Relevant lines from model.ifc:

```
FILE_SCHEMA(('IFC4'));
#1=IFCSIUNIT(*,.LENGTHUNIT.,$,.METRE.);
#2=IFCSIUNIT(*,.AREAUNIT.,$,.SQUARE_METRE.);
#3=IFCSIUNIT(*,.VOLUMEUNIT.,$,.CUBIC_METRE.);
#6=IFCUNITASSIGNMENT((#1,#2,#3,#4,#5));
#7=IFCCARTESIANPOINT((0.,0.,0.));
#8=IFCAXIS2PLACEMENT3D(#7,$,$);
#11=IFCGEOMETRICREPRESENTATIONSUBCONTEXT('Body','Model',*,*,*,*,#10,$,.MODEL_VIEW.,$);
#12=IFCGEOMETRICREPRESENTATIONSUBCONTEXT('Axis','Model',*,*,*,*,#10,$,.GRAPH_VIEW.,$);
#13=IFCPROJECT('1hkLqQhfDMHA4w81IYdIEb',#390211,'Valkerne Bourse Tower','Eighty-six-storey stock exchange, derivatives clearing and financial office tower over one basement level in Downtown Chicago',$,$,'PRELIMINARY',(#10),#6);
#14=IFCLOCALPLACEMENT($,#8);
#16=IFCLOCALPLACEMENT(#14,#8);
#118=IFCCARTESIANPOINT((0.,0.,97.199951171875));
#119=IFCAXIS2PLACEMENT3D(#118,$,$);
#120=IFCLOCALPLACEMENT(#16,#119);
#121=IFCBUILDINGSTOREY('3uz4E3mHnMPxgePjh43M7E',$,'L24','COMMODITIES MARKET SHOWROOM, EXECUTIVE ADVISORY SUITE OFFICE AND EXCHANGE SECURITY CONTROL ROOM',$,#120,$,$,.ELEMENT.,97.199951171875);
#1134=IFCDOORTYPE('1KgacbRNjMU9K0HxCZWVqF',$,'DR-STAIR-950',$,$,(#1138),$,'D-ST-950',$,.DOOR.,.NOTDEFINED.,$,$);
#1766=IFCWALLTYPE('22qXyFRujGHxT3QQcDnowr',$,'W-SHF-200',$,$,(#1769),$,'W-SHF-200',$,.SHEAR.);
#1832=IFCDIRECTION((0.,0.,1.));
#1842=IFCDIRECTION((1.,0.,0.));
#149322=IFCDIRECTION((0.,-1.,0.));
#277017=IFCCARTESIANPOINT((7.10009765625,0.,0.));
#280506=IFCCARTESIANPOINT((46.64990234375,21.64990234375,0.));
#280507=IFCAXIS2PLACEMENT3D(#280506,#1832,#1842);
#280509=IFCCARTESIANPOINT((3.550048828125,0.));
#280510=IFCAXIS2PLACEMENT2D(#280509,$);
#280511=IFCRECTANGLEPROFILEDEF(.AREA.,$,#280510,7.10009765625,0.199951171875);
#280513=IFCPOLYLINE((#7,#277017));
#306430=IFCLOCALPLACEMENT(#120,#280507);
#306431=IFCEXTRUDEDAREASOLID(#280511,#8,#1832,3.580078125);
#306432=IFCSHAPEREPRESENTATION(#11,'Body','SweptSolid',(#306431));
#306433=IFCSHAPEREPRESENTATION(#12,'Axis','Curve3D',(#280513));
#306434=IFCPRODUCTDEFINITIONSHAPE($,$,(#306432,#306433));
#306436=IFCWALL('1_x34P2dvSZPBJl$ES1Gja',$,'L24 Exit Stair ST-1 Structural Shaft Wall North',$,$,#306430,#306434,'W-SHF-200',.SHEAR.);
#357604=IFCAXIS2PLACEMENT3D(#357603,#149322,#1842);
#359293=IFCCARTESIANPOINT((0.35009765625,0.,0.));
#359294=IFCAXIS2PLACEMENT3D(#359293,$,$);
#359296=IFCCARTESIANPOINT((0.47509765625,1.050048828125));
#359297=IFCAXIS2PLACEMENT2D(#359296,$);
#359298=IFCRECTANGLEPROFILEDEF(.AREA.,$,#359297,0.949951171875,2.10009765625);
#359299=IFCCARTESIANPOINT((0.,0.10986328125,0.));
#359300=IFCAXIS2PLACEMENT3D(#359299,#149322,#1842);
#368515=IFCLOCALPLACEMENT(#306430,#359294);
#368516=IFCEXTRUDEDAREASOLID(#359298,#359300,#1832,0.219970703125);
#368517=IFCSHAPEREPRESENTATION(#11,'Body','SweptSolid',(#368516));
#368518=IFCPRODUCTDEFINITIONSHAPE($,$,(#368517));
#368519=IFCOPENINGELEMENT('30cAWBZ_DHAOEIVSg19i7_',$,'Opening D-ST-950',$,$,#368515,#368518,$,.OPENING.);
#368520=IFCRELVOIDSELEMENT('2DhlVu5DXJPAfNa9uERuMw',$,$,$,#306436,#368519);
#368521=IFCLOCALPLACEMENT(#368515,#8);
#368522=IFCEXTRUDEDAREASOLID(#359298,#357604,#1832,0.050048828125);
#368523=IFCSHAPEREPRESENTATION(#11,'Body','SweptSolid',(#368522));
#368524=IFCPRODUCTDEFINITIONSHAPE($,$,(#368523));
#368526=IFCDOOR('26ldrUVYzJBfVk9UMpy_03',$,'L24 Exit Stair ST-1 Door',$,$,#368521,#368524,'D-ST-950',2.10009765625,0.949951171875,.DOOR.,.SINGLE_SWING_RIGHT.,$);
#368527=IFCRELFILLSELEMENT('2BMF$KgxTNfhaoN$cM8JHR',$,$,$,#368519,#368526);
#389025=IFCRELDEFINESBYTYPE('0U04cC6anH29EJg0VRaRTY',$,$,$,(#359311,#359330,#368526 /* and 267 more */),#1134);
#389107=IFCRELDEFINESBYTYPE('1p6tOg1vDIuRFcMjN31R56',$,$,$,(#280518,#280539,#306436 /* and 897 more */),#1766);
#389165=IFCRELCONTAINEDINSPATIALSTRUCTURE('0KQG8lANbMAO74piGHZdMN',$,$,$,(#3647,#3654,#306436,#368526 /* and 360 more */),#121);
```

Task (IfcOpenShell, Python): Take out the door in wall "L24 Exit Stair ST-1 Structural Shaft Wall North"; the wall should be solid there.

```python
import ifcopenshell
import ifcopenshell.api.feature
import ifcopenshell.api.root
import ifcopenshell.geom
import ifcopenshell.util.shape

model = ifcopenshell.open("model.ifc")
settings = ifcopenshell.geom.settings()


def volume(element):
    """Net volume in cubic metres, openings subtracted."""
    shape = ifcopenshell.geom.create_shape(settings, element)
    return ifcopenshell.util.shape.get_volume(shape.geometry)


door = model.by_guid("26ldrUVYzJBfVk9UMpy_03")
opening = door.FillsVoids[0].RelatingOpeningElement
wall = opening.VoidsElements[0].RelatingBuildingElement
before = volume(wall)

ifcopenshell.api.root.remove_product(model, product=door)
ifcopenshell.api.feature.remove_feature(model, feature=opening)

after = volume(wall)

print(f"wall volume {before:.3f} -> {after:.3f} m3")

model.write("model-out.ifc")
```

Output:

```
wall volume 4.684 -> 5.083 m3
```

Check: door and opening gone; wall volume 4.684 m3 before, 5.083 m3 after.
